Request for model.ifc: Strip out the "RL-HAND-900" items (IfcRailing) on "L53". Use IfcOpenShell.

First a look at what the model holds.

```python
import ifcopenshell
import ifcopenshell.util.element

model = ifcopenshell.open("model.ifc")
print(model.schema)
storey = next(s for s in model.by_type("IfcBuildingStorey") if s.Name == "L53")
railings = [e for e in ifcopenshell.util.element.get_decomposition(storey) if e.is_a("IfcRailing")]
seen = {}
for e in railings:
    element_type = ifcopenshell.util.element.get_type(e)
    name = element_type.Name if element_type not in (None, e) else None
    seen[name] = seen.get(name, 0) + 1
for name, count in sorted(seen.items(), key=str):
    print(count, "x", name)
```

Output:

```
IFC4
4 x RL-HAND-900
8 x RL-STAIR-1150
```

```python
import ifcopenshell
import ifcopenshell.api.root
import ifcopenshell.util.element

model = ifcopenshell.open("model.ifc")

storey = next(s for s in model.by_type("IfcBuildingStorey") if s.Name == "L53")
railings = [e for e in ifcopenshell.util.element.get_decomposition(storey) if e.is_a("IfcRailing")]
targets = [e for e in railings if (t := ifcopenshell.util.element.get_type(e)) not in (None, e) and t.Name == "RL-HAND-900"]

for e in targets:
    ifcopenshell.api.root.remove_product(model, product=e)
print(len(targets), "removed")

model.write("model_rev.ifc")
```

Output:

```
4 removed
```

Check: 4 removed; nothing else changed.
